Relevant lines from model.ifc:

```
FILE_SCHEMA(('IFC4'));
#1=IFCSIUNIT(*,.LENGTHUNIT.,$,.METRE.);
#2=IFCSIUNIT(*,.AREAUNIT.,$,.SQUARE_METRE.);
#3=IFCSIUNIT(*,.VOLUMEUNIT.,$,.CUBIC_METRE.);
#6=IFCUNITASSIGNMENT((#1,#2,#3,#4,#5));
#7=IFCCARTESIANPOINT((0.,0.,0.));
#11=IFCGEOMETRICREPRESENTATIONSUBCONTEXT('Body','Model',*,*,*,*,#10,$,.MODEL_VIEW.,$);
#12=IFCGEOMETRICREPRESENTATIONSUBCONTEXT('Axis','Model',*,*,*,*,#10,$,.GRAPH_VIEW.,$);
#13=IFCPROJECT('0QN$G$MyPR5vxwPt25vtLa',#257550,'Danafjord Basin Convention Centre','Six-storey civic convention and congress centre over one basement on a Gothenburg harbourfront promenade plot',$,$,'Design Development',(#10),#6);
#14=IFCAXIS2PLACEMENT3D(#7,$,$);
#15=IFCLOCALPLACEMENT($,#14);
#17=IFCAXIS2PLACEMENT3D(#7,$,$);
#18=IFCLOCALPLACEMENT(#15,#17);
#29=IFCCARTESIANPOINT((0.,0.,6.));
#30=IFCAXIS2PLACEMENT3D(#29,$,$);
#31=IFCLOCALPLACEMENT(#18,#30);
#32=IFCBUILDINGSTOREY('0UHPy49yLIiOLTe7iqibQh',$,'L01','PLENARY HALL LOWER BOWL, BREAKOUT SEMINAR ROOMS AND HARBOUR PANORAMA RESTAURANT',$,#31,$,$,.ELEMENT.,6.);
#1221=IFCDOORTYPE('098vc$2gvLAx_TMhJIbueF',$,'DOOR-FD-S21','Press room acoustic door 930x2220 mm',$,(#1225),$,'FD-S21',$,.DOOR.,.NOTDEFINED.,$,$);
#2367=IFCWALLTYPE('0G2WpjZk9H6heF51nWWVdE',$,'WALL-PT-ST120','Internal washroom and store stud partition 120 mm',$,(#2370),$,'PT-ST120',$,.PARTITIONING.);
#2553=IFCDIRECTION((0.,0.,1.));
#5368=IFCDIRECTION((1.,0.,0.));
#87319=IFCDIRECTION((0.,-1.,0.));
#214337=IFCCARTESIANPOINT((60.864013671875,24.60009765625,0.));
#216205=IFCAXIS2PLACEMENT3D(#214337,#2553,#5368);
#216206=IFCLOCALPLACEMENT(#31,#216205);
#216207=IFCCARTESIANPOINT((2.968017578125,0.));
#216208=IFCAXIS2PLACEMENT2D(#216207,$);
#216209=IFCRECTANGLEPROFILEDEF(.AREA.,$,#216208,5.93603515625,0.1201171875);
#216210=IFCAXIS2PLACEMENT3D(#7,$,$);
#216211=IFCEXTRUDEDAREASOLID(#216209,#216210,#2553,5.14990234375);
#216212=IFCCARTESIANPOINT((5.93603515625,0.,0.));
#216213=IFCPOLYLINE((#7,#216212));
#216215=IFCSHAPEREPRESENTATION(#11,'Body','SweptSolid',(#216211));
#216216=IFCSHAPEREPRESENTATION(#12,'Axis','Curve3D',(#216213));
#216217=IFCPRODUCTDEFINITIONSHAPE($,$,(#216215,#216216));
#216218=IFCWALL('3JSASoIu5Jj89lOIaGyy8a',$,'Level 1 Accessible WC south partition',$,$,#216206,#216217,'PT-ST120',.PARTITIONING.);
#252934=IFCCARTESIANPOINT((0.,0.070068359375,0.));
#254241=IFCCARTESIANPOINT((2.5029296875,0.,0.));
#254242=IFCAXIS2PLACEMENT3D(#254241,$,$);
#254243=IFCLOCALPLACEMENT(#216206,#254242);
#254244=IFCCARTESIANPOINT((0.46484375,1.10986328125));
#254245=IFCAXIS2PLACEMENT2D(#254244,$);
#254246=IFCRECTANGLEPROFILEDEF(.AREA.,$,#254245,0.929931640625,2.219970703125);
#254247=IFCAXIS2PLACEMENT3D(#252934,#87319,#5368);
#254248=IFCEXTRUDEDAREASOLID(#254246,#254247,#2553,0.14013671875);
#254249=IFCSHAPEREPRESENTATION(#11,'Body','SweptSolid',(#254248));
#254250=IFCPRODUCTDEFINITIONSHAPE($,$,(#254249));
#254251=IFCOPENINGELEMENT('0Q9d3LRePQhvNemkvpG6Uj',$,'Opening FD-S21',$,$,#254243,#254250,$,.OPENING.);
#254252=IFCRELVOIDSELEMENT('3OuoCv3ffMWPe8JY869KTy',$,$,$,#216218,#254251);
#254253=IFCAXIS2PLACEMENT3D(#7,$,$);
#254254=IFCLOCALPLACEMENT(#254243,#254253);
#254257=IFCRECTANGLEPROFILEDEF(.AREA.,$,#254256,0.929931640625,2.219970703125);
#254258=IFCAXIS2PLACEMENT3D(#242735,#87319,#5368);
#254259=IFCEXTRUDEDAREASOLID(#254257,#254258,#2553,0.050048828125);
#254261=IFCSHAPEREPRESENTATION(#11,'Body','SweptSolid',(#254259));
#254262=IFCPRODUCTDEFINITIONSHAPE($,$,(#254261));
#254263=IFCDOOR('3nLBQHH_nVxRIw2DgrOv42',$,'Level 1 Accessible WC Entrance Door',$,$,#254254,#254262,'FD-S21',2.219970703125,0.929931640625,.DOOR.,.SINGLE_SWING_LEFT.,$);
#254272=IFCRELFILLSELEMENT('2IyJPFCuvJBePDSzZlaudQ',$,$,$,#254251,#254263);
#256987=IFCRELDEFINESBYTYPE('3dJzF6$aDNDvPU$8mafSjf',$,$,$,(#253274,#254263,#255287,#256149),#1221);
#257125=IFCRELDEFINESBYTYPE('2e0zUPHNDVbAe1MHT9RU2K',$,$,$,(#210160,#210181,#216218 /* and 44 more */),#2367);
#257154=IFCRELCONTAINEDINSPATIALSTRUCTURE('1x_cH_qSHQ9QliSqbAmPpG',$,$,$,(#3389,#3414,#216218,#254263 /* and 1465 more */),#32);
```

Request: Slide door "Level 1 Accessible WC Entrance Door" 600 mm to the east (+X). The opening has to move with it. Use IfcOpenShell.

```python
import ifcopenshell
import ifcopenshell.api.geometry
import ifcopenshell.util.placement

model = ifcopenshell.open("model.ifc")

door = model.by_id(254263)
opening = door.FillsVoids[0].RelatingOpeningElement
wall = opening.VoidsElements[0].RelatingBuildingElement

wall_matrix = ifcopenshell.util.placement.get_local_placement(wall.ObjectPlacement)
shift = wall_matrix[:3, 0] * 0.6
before = ifcopenshell.util.placement.get_local_placement(door.ObjectPlacement)[:3, 3].copy()

# The door is placed relative to its opening, so it follows when the opening moves.
matrix = ifcopenshell.util.placement.get_local_placement(opening.ObjectPlacement)
matrix[:3, 3] += shift
ifcopenshell.api.geometry.edit_object_placement(
    model, product=opening, matrix=matrix, is_si=False, should_transform_children=True
)

after = ifcopenshell.util.placement.get_local_placement(door.ObjectPlacement)[:3, 3]
print("door moved by", (after - before).round(3) + 0.0)

model.write("model_v2.ifc")
```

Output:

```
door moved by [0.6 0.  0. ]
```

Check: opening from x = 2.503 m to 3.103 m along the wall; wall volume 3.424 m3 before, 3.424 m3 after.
